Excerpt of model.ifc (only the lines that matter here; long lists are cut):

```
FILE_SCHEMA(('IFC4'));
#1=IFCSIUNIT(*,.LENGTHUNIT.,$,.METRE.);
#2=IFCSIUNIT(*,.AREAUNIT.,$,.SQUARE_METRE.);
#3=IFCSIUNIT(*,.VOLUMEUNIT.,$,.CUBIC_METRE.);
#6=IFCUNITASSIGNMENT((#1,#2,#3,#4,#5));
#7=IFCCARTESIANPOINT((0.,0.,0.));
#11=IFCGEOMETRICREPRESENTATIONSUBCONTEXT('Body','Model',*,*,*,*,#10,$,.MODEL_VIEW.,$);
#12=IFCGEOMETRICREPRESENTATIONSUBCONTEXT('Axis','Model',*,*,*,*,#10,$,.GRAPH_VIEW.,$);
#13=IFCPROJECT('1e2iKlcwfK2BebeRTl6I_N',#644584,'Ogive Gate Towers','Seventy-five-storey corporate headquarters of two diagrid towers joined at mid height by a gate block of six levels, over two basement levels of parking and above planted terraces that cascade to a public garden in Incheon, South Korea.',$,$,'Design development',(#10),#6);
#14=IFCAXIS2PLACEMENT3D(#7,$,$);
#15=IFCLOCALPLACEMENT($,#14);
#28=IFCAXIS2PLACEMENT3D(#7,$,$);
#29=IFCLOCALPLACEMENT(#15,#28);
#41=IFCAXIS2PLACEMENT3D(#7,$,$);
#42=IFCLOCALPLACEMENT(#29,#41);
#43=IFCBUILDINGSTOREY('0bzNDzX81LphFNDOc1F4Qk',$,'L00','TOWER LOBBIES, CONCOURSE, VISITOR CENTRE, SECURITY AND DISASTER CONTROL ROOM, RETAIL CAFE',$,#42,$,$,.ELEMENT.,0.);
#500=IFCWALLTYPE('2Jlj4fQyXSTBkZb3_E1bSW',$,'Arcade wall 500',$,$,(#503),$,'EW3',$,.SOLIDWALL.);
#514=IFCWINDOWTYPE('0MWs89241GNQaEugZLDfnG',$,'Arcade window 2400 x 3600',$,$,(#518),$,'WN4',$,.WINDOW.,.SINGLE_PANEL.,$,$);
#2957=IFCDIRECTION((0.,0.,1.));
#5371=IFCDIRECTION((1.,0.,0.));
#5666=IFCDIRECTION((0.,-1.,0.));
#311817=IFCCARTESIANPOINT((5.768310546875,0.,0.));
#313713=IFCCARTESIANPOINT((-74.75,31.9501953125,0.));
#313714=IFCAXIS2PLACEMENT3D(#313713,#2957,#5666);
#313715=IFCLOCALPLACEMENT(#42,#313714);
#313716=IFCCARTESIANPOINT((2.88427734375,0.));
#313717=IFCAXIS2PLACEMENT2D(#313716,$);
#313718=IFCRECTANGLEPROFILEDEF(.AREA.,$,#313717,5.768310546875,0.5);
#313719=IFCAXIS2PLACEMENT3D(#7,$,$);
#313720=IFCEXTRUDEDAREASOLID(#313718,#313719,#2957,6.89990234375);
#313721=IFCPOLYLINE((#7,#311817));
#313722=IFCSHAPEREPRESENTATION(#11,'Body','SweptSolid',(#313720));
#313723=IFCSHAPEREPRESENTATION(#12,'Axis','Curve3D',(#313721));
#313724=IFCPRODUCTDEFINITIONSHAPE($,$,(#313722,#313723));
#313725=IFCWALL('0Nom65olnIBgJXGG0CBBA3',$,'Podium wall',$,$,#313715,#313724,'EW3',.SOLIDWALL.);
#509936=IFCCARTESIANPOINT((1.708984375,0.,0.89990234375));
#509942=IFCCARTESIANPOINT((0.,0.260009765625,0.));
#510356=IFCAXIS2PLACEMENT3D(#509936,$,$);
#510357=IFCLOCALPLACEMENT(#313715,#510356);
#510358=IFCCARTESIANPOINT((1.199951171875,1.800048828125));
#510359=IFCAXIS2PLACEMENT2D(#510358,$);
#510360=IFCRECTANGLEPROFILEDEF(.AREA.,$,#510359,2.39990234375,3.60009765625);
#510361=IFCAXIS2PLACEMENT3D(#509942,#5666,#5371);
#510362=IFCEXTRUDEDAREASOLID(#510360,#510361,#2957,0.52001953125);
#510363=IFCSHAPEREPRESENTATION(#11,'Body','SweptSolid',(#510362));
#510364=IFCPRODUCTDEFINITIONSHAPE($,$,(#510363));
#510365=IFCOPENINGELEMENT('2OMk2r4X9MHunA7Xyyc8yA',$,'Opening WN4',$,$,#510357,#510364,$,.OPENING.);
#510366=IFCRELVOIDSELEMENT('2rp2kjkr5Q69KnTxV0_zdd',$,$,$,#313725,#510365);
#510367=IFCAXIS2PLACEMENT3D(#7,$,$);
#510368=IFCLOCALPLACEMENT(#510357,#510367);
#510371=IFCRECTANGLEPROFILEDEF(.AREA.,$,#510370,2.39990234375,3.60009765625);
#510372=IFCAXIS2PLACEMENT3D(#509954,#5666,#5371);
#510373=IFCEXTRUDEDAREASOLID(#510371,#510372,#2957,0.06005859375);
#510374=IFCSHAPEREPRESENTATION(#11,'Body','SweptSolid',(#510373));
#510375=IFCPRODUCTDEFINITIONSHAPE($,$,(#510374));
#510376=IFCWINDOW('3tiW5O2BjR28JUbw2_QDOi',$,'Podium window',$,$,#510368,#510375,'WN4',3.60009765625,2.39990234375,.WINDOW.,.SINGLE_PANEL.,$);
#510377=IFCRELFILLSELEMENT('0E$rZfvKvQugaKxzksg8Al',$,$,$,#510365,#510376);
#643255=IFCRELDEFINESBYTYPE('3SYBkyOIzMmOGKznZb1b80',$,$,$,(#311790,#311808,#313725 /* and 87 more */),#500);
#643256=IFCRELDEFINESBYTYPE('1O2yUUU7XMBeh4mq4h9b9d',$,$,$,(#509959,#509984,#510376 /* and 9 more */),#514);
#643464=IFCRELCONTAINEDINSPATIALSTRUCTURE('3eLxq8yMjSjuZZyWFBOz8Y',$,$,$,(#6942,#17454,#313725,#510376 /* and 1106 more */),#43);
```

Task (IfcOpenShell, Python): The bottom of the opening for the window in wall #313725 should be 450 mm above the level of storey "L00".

```python
import numpy as np
import ifcopenshell
import ifcopenshell.api.geometry
import ifcopenshell.geom
import ifcopenshell.util.element
import ifcopenshell.util.placement
import ifcopenshell.util.shape
import ifcopenshell.util.unit

model = ifcopenshell.open("model.ifc")
unit_scale = ifcopenshell.util.unit.calculate_unit_scale(model)

window = model.by_id(510376)
opening = window.FillsVoids[0].RelatingOpeningElement
storey = ifcopenshell.util.element.get_container(window, ifc_class="IfcBuildingStorey")
level = ifcopenshell.util.placement.get_local_placement(storey.ObjectPlacement)[2, 3]

# The opening's origin need not be at the sill, so measure its lowest point.
shape = ifcopenshell.geom.create_shape(ifcopenshell.geom.settings(), opening)
bottom = ifcopenshell.util.shape.get_shape_bottom_elevation(shape, shape.geometry) / unit_scale
dz = level + 0.45 / unit_scale - bottom

shift = np.array([0.0, 0.0, dz])
# The window is placed relative to its opening, so it follows when the opening moves.
matrix = ifcopenshell.util.placement.get_local_placement(opening.ObjectPlacement)
matrix[:3, 3] += shift
ifcopenshell.api.geometry.edit_object_placement(
    model, product=opening, matrix=matrix, is_si=False, should_transform_children=True
)

print(f"moved by {dz * unit_scale:+.3f} m")

model.write("model_v2.ifc")
```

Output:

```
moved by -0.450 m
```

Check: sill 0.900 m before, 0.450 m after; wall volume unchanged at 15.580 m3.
